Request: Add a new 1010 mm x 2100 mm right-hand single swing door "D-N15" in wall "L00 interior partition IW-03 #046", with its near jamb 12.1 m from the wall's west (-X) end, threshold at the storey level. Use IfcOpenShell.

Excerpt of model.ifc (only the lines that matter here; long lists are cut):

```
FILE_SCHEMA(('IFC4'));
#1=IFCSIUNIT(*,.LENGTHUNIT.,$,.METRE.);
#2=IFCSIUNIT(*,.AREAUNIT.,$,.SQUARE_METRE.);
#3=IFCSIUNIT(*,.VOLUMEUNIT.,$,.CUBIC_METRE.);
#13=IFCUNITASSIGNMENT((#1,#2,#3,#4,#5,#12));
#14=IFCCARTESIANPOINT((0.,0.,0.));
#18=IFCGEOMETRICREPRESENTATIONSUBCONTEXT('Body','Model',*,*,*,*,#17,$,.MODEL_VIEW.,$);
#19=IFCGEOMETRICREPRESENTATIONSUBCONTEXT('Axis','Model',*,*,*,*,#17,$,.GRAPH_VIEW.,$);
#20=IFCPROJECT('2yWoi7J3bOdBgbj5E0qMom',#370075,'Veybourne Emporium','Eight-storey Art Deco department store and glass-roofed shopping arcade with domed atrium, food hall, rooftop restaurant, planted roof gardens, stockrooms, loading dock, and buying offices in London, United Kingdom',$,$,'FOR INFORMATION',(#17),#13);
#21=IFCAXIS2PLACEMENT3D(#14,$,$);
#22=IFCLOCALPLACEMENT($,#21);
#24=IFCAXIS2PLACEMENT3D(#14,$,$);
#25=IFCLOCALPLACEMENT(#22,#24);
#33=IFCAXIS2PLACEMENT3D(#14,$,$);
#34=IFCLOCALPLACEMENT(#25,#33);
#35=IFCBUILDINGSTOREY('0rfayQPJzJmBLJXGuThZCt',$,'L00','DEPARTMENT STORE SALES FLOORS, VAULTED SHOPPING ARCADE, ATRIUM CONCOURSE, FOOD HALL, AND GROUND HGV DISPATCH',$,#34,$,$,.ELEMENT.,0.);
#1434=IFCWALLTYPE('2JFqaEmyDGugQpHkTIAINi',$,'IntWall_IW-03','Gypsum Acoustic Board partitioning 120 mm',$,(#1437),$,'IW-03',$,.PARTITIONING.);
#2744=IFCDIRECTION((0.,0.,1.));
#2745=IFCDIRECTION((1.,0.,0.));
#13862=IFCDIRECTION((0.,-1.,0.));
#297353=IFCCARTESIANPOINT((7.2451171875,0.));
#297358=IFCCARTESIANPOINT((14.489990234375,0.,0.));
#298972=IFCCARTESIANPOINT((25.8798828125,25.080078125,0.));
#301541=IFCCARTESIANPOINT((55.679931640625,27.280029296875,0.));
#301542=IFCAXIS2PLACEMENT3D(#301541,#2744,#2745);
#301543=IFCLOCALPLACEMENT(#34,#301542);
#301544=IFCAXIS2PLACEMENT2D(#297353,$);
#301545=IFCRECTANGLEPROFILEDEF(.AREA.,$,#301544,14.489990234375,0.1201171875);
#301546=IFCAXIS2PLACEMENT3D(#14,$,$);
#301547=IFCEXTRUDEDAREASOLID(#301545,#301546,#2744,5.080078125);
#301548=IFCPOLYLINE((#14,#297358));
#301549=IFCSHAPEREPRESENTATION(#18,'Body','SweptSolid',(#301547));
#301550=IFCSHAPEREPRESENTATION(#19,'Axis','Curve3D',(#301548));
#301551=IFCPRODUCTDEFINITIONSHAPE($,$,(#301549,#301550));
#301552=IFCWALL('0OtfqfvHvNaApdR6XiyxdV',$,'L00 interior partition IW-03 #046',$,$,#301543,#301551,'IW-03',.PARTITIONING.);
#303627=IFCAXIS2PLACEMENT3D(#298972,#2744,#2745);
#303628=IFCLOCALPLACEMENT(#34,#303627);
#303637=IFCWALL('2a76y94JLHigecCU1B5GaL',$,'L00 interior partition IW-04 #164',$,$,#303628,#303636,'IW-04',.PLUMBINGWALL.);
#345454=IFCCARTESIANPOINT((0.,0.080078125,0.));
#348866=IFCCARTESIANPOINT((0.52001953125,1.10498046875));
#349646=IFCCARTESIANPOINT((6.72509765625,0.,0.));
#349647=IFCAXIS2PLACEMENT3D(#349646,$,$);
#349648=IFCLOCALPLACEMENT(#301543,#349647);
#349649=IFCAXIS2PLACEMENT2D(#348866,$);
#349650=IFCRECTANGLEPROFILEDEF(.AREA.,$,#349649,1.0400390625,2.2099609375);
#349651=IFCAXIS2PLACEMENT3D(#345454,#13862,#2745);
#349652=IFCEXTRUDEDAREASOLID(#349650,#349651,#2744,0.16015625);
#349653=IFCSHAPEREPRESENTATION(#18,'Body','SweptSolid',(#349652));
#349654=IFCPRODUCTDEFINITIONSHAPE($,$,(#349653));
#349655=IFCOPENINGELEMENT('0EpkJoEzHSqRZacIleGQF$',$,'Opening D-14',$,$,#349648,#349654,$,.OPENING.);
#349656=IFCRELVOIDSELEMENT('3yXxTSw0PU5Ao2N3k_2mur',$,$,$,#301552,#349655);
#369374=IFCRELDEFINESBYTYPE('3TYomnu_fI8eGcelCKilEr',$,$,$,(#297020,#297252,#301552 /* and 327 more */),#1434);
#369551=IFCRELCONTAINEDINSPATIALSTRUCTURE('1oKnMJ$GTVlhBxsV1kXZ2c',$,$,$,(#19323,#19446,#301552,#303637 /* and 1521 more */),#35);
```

```python
import numpy as np
import ifcopenshell
import ifcopenshell.api.feature
import ifcopenshell.api.geometry
import ifcopenshell.api.root
import ifcopenshell.api.spatial
import ifcopenshell.geom
import ifcopenshell.util.element
import ifcopenshell.util.placement
import ifcopenshell.util.representation
import ifcopenshell.util.shape
import ifcopenshell.util.unit

model = ifcopenshell.open("model.ifc")
unit_scale = ifcopenshell.util.unit.calculate_unit_scale(model)
settings = ifcopenshell.geom.settings()


def volume(element):
    """Net volume in cubic metres, openings subtracted."""
    shape = ifcopenshell.geom.create_shape(settings, element)
    return ifcopenshell.util.shape.get_volume(shape.geometry)


wall = model.by_guid("0OtfqfvHvNaApdR6XiyxdV")
storey = ifcopenshell.util.element.get_container(wall, ifc_class="IfcBuildingStorey")
context = ifcopenshell.util.representation.get_context(model, "Model", "Body", "MODEL_VIEW")
before = volume(wall)

width, height, from_end, sill = 1.01, 2.1, 12.1, 0.0  # metres

# The wall runs along its own X axis, and the end named is its -X end.
wall_shape = ifcopenshell.geom.create_shape(settings, wall)
x, y, z = ifcopenshell.util.shape.get_vertices(wall_shape.geometry).T
start = x.min() + from_end
face, thickness = float(y.min()), float(y.max() - y.min())
wall_matrix = ifcopenshell.util.placement.get_local_placement(wall.ObjectPlacement)
level = ifcopenshell.util.placement.get_local_placement(storey.ObjectPlacement)[2, 3]


def in_wall(x, y):
    """Placement at x, y metres in the wall's axes, at sill height."""
    matrix = wall_matrix.copy()
    matrix[:, 3] = wall_matrix @ np.array([x / unit_scale, y / unit_scale, 0.0, 1.0])
    matrix[2, 3] = level + sill / unit_scale
    return matrix


# Opening: a box that overshoots both wall faces by 50 mm.
opening = ifcopenshell.api.root.create_entity(model, ifc_class="IfcOpeningElement", predefined_type="OPENING")
box = ifcopenshell.api.geometry.add_wall_representation(
    model, context=context, length=width, height=height, thickness=thickness + 0.1
)
ifcopenshell.api.geometry.assign_representation(model, product=opening, representation=box)
ifcopenshell.api.geometry.edit_object_placement(model, product=opening, matrix=in_wall(start, face - 0.05), is_si=False)
ifcopenshell.api.feature.add_feature(model, feature=opening, element=wall)

door = ifcopenshell.api.root.create_entity(model, ifc_class="IfcDoor", name="D-N15", predefined_type="DOOR")
door.OverallWidth, door.OverallHeight = width / unit_scale, height / unit_scale
door.OperationType = "SINGLE_SWING_RIGHT"
body = ifcopenshell.api.geometry.add_door_representation(
    model,
    context=context,
    overall_width=door.OverallWidth,
    overall_height=door.OverallHeight,
    operation_type="SINGLE_SWING_RIGHT",
    lining_properties={"LiningDepth": thickness / unit_scale, "ThresholdDepth": thickness / unit_scale},
)
ifcopenshell.api.geometry.assign_representation(model, product=door, representation=body)
ifcopenshell.api.spatial.assign_container(model, products=[door], relating_structure=storey)
ifcopenshell.api.feature.add_filling(model, opening=opening, element=door)

# The lining spans the wall, so the door starts at the wall face.
ifcopenshell.api.geometry.edit_object_placement(model, product=door, matrix=in_wall(start, face), is_si=False)

after = volume(wall)

print(f"wall volume {before:.3f} -> {after:.3f} m3")

model.write("model_v2.ifc")
```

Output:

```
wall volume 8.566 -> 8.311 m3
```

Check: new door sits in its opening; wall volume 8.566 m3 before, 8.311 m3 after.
